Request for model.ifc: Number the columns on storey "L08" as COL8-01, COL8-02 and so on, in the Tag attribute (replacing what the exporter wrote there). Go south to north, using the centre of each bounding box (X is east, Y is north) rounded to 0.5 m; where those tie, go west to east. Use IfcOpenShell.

First a look at what the model holds.

```python
import ifcopenshell
import ifcopenshell.util.element
import ifcopenshell.util.placement

model = ifcopenshell.open("model.ifc")
print(model.schema)
storey = next(s for s in model.by_type("IfcBuildingStorey") if s.Name == "L08")
columns = [e for e in ifcopenshell.util.element.get_decomposition(storey) if e.is_a("IfcColumn")]
for e in sorted(columns, key=lambda e: e.id()):
    origin = ifcopenshell.util.placement.get_local_placement(e.ObjectPlacement)[:3, 3]
    print(e.id(), e.Tag, e.Name, origin.round(2) + 0.0, sep=" | ")
```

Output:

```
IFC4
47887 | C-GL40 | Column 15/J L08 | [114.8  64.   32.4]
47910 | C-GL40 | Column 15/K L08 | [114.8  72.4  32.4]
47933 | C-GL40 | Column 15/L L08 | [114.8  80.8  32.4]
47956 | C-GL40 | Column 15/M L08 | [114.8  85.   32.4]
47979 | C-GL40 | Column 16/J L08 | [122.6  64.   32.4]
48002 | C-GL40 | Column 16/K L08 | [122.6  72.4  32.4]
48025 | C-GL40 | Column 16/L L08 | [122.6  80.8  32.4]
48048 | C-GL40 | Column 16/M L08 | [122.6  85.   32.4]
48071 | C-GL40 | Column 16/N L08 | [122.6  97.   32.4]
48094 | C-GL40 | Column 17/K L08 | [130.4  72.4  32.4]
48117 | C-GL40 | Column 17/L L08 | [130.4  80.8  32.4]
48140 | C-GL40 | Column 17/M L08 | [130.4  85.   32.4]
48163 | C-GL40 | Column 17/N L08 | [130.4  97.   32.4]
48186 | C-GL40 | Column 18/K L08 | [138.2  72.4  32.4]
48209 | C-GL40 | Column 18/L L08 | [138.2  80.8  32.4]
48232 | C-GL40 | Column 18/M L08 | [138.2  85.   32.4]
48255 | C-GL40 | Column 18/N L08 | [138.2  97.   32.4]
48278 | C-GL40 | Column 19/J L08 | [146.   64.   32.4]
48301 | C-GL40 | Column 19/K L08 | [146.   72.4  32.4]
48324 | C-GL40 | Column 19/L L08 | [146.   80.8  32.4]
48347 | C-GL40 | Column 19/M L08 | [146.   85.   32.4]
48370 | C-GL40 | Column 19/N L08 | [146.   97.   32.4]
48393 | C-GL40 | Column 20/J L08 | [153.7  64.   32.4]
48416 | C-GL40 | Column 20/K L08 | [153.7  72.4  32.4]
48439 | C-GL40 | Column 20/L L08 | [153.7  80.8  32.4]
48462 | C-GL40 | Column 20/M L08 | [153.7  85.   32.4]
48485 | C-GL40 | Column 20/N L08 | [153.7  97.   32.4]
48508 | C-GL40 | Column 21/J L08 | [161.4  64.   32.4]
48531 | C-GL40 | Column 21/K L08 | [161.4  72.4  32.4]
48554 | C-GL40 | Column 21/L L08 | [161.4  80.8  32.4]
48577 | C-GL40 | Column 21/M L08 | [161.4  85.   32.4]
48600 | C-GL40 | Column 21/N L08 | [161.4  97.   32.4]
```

```python
import ifcopenshell
import ifcopenshell.geom
import ifcopenshell.util.element
import ifcopenshell.util.shape

model = ifcopenshell.open("model.ifc")
settings = ifcopenshell.geom.settings()
settings.set("use-world-coords", True)


def centre(element):
    shape = ifcopenshell.geom.create_shape(settings, element)
    return ifcopenshell.util.shape.get_bbox_centroid(shape.geometry)


storey = next(s for s in model.by_type("IfcBuildingStorey") if s.Name == "L08")
columns = [e for e in ifcopenshell.util.element.get_decomposition(storey) if e.is_a("IfcColumn")]

# Insertion points can sit at a corner or the storey origin, so sort by the geometry (in metres).
centres = {e: centre(e) for e in columns}
columns.sort(key=lambda e: (round(centres[e][1] / 0.5), centres[e][0]))

for i, e in enumerate(columns, start=1):
    number = f"COL8-{i:02d}"
    e.Tag = number
    print(e.id(), number)

model.write("model-out.ifc")
```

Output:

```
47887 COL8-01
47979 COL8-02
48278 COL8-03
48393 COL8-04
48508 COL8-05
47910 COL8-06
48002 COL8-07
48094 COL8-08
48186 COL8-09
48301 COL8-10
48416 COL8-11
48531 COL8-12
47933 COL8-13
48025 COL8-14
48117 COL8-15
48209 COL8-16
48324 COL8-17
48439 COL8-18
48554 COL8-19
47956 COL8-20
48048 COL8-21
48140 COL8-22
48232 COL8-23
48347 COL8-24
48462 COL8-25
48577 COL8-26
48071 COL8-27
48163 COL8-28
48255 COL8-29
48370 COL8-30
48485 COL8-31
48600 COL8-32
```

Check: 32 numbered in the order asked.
